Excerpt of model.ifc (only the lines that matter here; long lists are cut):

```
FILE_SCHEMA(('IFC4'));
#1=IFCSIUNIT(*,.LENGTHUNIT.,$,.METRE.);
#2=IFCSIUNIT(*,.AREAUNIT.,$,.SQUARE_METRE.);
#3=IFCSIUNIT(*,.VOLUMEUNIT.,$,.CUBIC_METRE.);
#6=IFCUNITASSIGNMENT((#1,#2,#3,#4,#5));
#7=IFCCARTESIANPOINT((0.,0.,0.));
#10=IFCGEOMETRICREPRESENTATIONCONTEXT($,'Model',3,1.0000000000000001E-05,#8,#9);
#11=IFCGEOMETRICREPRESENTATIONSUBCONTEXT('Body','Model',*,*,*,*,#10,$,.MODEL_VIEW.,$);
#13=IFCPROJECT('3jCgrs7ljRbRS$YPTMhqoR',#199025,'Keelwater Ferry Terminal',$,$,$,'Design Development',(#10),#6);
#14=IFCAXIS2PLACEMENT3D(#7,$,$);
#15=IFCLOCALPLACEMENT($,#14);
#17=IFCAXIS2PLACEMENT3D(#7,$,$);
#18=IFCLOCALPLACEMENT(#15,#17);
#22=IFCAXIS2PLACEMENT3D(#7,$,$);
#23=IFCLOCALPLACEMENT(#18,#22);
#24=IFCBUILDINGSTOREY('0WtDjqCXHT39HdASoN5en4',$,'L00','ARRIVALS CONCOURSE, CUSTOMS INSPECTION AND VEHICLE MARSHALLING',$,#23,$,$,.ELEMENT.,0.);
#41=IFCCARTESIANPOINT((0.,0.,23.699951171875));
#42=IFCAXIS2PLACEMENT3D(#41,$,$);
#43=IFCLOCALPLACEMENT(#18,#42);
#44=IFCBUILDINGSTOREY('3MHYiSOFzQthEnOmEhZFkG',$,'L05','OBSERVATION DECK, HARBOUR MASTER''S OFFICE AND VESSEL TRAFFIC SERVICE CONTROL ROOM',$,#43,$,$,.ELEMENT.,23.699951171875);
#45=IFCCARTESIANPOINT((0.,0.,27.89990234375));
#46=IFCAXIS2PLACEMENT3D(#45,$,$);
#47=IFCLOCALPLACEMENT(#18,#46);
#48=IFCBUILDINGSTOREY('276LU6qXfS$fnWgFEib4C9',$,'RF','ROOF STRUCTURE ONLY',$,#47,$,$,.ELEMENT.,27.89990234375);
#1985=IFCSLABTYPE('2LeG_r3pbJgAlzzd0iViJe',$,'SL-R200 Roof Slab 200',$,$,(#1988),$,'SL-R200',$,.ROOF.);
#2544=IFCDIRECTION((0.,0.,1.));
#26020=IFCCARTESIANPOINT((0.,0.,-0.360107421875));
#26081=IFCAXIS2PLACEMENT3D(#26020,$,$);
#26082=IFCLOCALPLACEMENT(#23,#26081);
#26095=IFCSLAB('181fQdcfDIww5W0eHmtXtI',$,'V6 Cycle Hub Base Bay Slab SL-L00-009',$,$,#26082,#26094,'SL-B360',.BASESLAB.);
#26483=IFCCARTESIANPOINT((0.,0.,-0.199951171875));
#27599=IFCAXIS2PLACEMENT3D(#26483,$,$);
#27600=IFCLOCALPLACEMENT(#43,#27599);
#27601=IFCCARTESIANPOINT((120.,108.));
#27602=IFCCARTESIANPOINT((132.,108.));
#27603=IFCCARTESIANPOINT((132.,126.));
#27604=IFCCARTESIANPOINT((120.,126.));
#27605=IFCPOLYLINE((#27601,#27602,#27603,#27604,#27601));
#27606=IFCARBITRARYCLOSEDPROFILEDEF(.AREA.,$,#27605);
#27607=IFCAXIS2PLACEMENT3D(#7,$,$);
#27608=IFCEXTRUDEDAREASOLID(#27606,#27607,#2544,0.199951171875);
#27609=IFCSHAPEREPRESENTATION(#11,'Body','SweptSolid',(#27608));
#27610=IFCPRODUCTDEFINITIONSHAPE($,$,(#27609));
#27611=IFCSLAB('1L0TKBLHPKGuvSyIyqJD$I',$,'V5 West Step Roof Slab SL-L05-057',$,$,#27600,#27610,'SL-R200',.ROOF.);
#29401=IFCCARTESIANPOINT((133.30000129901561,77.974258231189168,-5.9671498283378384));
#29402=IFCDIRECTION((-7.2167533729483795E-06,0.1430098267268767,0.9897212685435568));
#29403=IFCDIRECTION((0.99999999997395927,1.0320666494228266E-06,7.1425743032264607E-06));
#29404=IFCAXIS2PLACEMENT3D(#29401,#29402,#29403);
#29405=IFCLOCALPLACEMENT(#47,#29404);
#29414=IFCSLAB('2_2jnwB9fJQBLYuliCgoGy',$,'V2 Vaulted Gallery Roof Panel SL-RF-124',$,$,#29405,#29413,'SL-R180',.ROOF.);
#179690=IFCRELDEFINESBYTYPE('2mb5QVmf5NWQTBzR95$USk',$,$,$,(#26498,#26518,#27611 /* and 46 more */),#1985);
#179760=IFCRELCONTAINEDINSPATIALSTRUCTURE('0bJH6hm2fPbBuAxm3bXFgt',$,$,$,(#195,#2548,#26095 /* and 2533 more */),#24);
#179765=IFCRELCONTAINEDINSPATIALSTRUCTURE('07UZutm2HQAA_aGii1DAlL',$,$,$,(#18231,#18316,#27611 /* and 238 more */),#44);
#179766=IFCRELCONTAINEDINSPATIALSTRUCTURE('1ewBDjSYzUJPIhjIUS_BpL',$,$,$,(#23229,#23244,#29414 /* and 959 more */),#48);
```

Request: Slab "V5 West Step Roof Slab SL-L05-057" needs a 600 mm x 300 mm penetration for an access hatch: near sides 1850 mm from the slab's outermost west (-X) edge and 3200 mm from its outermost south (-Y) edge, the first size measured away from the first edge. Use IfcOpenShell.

```python
import numpy as np
import ifcopenshell
import ifcopenshell.api.feature
import ifcopenshell.api.geometry
import ifcopenshell.api.root
import ifcopenshell.geom
import ifcopenshell.util.placement
import ifcopenshell.util.representation
import ifcopenshell.util.shape
import ifcopenshell.util.unit

model = ifcopenshell.open("model.ifc")
unit_scale = ifcopenshell.util.unit.calculate_unit_scale(model)
settings = ifcopenshell.geom.settings()


def volume(element):
    """Net volume in cubic metres, openings subtracted."""
    shape = ifcopenshell.geom.create_shape(settings, element)
    return ifcopenshell.util.shape.get_volume(shape.geometry)


slab = model.by_guid("1L0TKBLHPKGuvSyIyqJD$I")
before = volume(slab)

# Extent in the slab's own axes, in metres. The edges named are its -X and -Y sides.
slab_shape = ifcopenshell.geom.create_shape(settings, slab)
vertices = ifcopenshell.util.shape.get_vertices(slab_shape.geometry)
x_min, y_min, bottom = vertices.min(axis=0)
top = vertices[:, 2].max()

opening = ifcopenshell.api.root.create_entity(model, ifc_class="IfcOpeningElement", name="Access hatch opening", predefined_type="OPENING")
context = ifcopenshell.util.representation.get_context(model, "Model", "Body", "MODEL_VIEW")
width, depth = 0.6, 0.3
outline = [(0.0, 0.0), (width, 0.0), (width, depth), (0.0, depth), (0.0, 0.0)]
# Overshoot both faces by 50 mm so the cut is clean.
shape = ifcopenshell.api.geometry.add_slab_representation(
    model, context=context, depth=top - bottom + 0.1, polyline=outline
)
ifcopenshell.api.geometry.assign_representation(model, product=opening, representation=shape)

matrix = ifcopenshell.util.placement.get_local_placement(slab.ObjectPlacement)
matrix[:, 3] = matrix @ np.append(np.array([x_min + 1.85, y_min + 3.2, bottom - 0.05]) / unit_scale, 1.0)
ifcopenshell.api.geometry.edit_object_placement(model, product=opening, matrix=matrix, is_si=False)
ifcopenshell.api.feature.add_feature(model, feature=opening, element=slab)

after = volume(slab)

print(f"slab volume {before:.3f} -> {after:.3f} m3")

model.write("model_v2.ifc")
```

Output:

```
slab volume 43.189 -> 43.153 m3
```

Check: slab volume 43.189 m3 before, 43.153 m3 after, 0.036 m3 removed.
